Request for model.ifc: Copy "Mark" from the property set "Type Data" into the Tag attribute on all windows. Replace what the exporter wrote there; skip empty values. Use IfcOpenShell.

First a look at what the model holds.

```python
import ifcopenshell
import ifcopenshell.util.element

model = ifcopenshell.open("model.ifc")
print(model.schema)
windows = model.by_type("IfcWindow")
print(len(windows), "windows")
for e in windows[:8]:
    source = ifcopenshell.util.element.get_pset(e, "Type Data", "Mark")
    target = e.Tag
    print(e.id(), repr(source), repr(target), sep=" | ")
```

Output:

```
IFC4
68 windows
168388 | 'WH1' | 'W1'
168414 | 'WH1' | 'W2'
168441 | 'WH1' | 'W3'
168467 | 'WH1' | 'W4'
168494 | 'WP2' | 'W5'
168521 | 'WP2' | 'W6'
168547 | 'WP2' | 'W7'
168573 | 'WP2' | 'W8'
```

```python
import ifcopenshell
import ifcopenshell.util.element

model = ifcopenshell.open("model.ifc")

count = 0
for e in model.by_type("IfcWindow"):
    value = ifcopenshell.util.element.get_pset(e, "Type Data", "Mark")
    current = e.Tag
    if not value or not value.strip() or current == value:
        continue
    e.Tag = value
    count += 1

print(count, "windows updated")

model.write("model_edited.ifc")
```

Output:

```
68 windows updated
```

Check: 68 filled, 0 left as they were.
